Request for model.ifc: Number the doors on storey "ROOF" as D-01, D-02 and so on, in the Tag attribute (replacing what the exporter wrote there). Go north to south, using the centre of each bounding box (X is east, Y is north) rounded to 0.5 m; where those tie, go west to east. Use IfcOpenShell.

First a look at what the model holds.

```python
import ifcopenshell
import ifcopenshell.util.element
import ifcopenshell.util.placement

model = ifcopenshell.open("model.ifc")
print(model.schema)
storey = next(s for s in model.by_type("IfcBuildingStorey") if s.Name == "ROOF")
doors = [e for e in ifcopenshell.util.element.get_decomposition(storey) if e.is_a("IfcDoor")]
for e in sorted(doors, key=lambda e: e.id()):
    origin = ifcopenshell.util.placement.get_local_placement(e.ObjectPlacement)[:3, 3]
    print(e.id(), e.Tag, e.Name, origin.round(2) + 0.0, sep=" | ")
```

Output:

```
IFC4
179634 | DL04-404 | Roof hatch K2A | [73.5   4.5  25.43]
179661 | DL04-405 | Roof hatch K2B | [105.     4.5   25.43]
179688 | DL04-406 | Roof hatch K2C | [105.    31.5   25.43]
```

```python
import ifcopenshell
import ifcopenshell.geom
import ifcopenshell.util.element
import ifcopenshell.util.shape

model = ifcopenshell.open("model.ifc")
settings = ifcopenshell.geom.settings()
settings.set("use-world-coords", True)


def centre(element):
    shape = ifcopenshell.geom.create_shape(settings, element)
    return ifcopenshell.util.shape.get_bbox_centroid(shape.geometry)


storey = next(s for s in model.by_type("IfcBuildingStorey") if s.Name == "ROOF")
doors = [e for e in ifcopenshell.util.element.get_decomposition(storey) if e.is_a("IfcDoor")]

# Insertion points can sit at a corner or the storey origin, so sort by the geometry (in metres).
centres = {e: centre(e) for e in doors}
doors.sort(key=lambda e: (-round(centres[e][1] / 0.5), centres[e][0]))

for i, e in enumerate(doors, start=1):
    number = f"D-{i:02d}"
    e.Tag = number
    print(e.id(), number)

model.write("model_v2.ifc")
```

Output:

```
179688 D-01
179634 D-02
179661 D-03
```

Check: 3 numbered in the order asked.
